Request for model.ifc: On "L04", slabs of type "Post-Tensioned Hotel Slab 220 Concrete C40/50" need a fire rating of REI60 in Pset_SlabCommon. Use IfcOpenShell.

First a look at what the model holds.

```python
import ifcopenshell
import ifcopenshell.util.element

model = ifcopenshell.open("model.ifc")
print(model.schema)
storey = next(s for s in model.by_type("IfcBuildingStorey") if s.Name == "L04")
slabs = [e for e in ifcopenshell.util.element.get_decomposition(storey) if e.is_a("IfcSlab")]
seen = {}
for e in slabs:
    element_type = ifcopenshell.util.element.get_type(e)
    key = (element_type.Name if element_type != e and element_type else None, ifcopenshell.util.element.get_pset(e, "Pset_SlabCommon", "FireRating"))
    seen[key] = seen.get(key, 0) + 1
for (name, value), count in sorted(seen.items(), key=str):
    print(count, "x", name, "|", value)
```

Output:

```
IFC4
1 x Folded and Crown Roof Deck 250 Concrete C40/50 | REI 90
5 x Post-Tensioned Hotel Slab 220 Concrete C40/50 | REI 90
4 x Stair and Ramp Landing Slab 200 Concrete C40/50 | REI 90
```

```python
import ifcopenshell
import ifcopenshell.api.pset
import ifcopenshell.util.element

model = ifcopenshell.open("model.ifc")

storey = next(s for s in model.by_type("IfcBuildingStorey") if s.Name == "L04")
slabs = [e for e in ifcopenshell.util.element.get_decomposition(storey) if e.is_a("IfcSlab")]

count = 0
for e in slabs:
    element_type = ifcopenshell.util.element.get_type(e)
    if element_type in (None, e) or element_type.Name != "Post-Tensioned Hotel Slab 220 Concrete C40/50":
        continue
    # add_pset returns the element's existing set when there is one.
    pset = ifcopenshell.api.pset.add_pset(model, product=e, name="Pset_SlabCommon")
    ifcopenshell.api.pset.edit_pset(model, pset=pset, properties={"FireRating": "REI60"})
    count += 1

print(count, "slabs updated")

model.write("model_edited.ifc")
```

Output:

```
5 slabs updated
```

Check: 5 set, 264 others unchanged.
